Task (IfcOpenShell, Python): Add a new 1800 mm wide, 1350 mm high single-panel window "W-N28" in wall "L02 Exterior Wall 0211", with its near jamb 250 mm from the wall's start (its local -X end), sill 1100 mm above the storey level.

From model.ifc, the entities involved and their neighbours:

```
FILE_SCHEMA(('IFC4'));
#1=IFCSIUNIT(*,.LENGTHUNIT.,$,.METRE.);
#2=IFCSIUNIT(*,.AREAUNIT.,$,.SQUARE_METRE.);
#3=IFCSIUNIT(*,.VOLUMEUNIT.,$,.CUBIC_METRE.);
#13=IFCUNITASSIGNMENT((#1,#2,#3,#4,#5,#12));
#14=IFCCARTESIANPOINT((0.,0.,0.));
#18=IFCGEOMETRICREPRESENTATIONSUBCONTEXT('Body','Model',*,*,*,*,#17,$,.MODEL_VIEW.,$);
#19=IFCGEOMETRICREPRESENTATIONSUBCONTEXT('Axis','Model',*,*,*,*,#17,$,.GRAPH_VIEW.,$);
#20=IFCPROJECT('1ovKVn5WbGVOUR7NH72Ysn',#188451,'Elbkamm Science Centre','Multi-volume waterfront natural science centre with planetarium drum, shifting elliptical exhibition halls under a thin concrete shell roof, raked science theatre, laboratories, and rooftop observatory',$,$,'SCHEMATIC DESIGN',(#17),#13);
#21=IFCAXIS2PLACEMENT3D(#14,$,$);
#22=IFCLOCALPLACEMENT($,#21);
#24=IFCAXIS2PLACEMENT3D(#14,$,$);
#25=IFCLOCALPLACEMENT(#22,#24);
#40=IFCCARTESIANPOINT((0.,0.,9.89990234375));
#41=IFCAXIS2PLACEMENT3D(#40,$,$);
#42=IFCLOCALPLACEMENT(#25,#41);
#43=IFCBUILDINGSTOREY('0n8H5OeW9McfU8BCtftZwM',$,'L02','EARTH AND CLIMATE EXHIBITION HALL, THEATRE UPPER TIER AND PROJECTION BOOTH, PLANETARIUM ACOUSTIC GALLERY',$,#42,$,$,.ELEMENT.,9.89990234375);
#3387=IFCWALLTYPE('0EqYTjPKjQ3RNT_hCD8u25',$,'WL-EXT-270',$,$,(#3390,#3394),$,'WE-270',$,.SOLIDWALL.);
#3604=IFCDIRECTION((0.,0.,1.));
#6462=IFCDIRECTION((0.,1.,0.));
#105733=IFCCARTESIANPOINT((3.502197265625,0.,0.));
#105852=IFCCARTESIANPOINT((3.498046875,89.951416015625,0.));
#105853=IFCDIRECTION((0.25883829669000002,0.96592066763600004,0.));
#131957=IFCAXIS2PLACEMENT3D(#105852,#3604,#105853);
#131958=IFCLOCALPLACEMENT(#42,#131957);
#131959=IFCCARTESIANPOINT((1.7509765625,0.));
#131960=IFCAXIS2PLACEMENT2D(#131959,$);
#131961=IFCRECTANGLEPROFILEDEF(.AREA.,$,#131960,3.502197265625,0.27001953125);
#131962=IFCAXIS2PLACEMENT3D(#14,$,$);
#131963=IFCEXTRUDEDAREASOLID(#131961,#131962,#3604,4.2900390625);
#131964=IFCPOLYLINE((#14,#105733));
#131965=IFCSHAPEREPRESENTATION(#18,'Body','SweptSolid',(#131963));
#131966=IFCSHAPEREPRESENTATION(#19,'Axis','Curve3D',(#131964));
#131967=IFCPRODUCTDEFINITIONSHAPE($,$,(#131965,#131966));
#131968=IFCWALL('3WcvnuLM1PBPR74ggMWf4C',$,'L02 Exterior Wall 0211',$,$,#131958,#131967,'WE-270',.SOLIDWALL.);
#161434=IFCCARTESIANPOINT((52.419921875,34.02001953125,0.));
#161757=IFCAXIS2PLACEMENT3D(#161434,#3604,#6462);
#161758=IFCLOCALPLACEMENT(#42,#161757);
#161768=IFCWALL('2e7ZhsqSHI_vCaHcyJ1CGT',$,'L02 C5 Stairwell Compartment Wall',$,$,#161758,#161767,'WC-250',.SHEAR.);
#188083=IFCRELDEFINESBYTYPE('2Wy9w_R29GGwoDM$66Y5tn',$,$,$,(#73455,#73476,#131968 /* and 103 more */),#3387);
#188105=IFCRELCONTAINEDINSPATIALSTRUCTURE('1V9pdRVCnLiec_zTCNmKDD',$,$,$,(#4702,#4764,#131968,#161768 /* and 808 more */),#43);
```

```python
import numpy as np
import ifcopenshell
import ifcopenshell.api.feature
import ifcopenshell.api.geometry
import ifcopenshell.api.root
import ifcopenshell.api.spatial
import ifcopenshell.geom
import ifcopenshell.util.element
import ifcopenshell.util.placement
import ifcopenshell.util.representation
import ifcopenshell.util.shape
import ifcopenshell.util.unit

model = ifcopenshell.open("model.ifc")
unit_scale = ifcopenshell.util.unit.calculate_unit_scale(model)
settings = ifcopenshell.geom.settings()


def volume(element):
    """Net volume in cubic metres, openings subtracted."""
    shape = ifcopenshell.geom.create_shape(settings, element)
    return ifcopenshell.util.shape.get_volume(shape.geometry)


wall = model.by_id(131968)
storey = ifcopenshell.util.element.get_container(wall, ifc_class="IfcBuildingStorey")
context = ifcopenshell.util.representation.get_context(model, "Model", "Body", "MODEL_VIEW")
before = volume(wall)

width, height, from_end, sill = 1.8, 1.35, 0.25, 1.1  # metres

# The wall runs along its own X axis, and the end named is its -X end.
wall_shape = ifcopenshell.geom.create_shape(settings, wall)
x, y, z = ifcopenshell.util.shape.get_vertices(wall_shape.geometry).T
start = x.min() + from_end
face, thickness = float(y.min()), float(y.max() - y.min())
wall_matrix = ifcopenshell.util.placement.get_local_placement(wall.ObjectPlacement)
level = ifcopenshell.util.placement.get_local_placement(storey.ObjectPlacement)[2, 3]


def in_wall(x, y):
    """Placement at x, y metres in the wall's axes, at sill height."""
    matrix = wall_matrix.copy()
    matrix[:, 3] = wall_matrix @ np.array([x / unit_scale, y / unit_scale, 0.0, 1.0])
    matrix[2, 3] = level + sill / unit_scale
    return matrix


# Opening: a box that overshoots both wall faces by 50 mm.
opening = ifcopenshell.api.root.create_entity(model, ifc_class="IfcOpeningElement", predefined_type="OPENING")
box = ifcopenshell.api.geometry.add_wall_representation(
    model, context=context, length=width, height=height, thickness=thickness + 0.1
)
ifcopenshell.api.geometry.assign_representation(model, product=opening, representation=box)
ifcopenshell.api.geometry.edit_object_placement(model, product=opening, matrix=in_wall(start, face - 0.05), is_si=False)
ifcopenshell.api.feature.add_feature(model, feature=opening, element=wall)

window = ifcopenshell.api.root.create_entity(model, ifc_class="IfcWindow", name="W-N28", predefined_type="WINDOW")
window.OverallWidth, window.OverallHeight = width / unit_scale, height / unit_scale
window.PartitioningType = "SINGLE_PANEL"
body = ifcopenshell.api.geometry.add_window_representation(
    model,
    context=context,
    overall_width=window.OverallWidth,
    overall_height=window.OverallHeight,
    partition_type="SINGLE_PANEL",
)
ifcopenshell.api.geometry.assign_representation(model, product=window, representation=body)
ifcopenshell.api.spatial.assign_container(model, products=[window], relating_structure=storey)
ifcopenshell.api.feature.add_filling(model, opening=opening, element=window)

# Centre the window in the wall's thickness.
ifcopenshell.api.geometry.edit_object_placement(model, product=window, matrix=in_wall(start, face), is_si=False)
window_shape = ifcopenshell.geom.create_shape(settings, window)
depth = ifcopenshell.util.shape.get_vertices(window_shape.geometry)[:, 1]
offset = face + thickness / 2 - (depth.min() + depth.max()) / 2
ifcopenshell.api.geometry.edit_object_placement(model, product=window, matrix=in_wall(start, offset), is_si=False)

after = volume(wall)

print(f"wall volume {before:.3f} -> {after:.3f} m3")

model.write("model_updated.ifc")
```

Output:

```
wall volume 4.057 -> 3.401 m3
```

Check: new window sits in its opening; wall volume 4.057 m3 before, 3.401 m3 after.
